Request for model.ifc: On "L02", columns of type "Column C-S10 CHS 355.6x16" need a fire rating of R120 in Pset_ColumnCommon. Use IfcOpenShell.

First a look at what the model holds.

```python
import ifcopenshell
import ifcopenshell.util.element

model = ifcopenshell.open("model.ifc")
print(model.schema)
storey = next(s for s in model.by_type("IfcBuildingStorey") if s.Name == "L02")
columns = [e for e in ifcopenshell.util.element.get_decomposition(storey) if e.is_a("IfcColumn")]
seen = {}
for e in columns:
    element_type = ifcopenshell.util.element.get_type(e)
    key = (element_type.Name if element_type != e and element_type else None, ifcopenshell.util.element.get_pset(e, "Pset_ColumnCommon", "FireRating"))
    seen[key] = seen.get(key, 0) + 1
for (name, value), count in sorted(seen.items(), key=str):
    print(count, "x", name, "|", value)
```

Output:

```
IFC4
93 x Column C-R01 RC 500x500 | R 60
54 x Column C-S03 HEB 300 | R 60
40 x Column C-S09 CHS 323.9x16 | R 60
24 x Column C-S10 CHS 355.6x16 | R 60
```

```python
import ifcopenshell
import ifcopenshell.api.pset
import ifcopenshell.util.element

model = ifcopenshell.open("model.ifc")

storey = next(s for s in model.by_type("IfcBuildingStorey") if s.Name == "L02")
columns = [e for e in ifcopenshell.util.element.get_decomposition(storey) if e.is_a("IfcColumn")]

count = 0
for e in columns:
    element_type = ifcopenshell.util.element.get_type(e)
    if element_type in (None, e) or element_type.Name != "Column C-S10 CHS 355.6x16":
        continue
    # add_pset returns the element's existing set when there is one.
    pset = ifcopenshell.api.pset.add_pset(model, product=e, name="Pset_ColumnCommon")
    ifcopenshell.api.pset.edit_pset(model, pset=pset, properties={"FireRating": "R120"})
    count += 1

print(count, "columns updated")

model.write("model_v2.ifc")
```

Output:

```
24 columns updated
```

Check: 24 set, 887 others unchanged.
